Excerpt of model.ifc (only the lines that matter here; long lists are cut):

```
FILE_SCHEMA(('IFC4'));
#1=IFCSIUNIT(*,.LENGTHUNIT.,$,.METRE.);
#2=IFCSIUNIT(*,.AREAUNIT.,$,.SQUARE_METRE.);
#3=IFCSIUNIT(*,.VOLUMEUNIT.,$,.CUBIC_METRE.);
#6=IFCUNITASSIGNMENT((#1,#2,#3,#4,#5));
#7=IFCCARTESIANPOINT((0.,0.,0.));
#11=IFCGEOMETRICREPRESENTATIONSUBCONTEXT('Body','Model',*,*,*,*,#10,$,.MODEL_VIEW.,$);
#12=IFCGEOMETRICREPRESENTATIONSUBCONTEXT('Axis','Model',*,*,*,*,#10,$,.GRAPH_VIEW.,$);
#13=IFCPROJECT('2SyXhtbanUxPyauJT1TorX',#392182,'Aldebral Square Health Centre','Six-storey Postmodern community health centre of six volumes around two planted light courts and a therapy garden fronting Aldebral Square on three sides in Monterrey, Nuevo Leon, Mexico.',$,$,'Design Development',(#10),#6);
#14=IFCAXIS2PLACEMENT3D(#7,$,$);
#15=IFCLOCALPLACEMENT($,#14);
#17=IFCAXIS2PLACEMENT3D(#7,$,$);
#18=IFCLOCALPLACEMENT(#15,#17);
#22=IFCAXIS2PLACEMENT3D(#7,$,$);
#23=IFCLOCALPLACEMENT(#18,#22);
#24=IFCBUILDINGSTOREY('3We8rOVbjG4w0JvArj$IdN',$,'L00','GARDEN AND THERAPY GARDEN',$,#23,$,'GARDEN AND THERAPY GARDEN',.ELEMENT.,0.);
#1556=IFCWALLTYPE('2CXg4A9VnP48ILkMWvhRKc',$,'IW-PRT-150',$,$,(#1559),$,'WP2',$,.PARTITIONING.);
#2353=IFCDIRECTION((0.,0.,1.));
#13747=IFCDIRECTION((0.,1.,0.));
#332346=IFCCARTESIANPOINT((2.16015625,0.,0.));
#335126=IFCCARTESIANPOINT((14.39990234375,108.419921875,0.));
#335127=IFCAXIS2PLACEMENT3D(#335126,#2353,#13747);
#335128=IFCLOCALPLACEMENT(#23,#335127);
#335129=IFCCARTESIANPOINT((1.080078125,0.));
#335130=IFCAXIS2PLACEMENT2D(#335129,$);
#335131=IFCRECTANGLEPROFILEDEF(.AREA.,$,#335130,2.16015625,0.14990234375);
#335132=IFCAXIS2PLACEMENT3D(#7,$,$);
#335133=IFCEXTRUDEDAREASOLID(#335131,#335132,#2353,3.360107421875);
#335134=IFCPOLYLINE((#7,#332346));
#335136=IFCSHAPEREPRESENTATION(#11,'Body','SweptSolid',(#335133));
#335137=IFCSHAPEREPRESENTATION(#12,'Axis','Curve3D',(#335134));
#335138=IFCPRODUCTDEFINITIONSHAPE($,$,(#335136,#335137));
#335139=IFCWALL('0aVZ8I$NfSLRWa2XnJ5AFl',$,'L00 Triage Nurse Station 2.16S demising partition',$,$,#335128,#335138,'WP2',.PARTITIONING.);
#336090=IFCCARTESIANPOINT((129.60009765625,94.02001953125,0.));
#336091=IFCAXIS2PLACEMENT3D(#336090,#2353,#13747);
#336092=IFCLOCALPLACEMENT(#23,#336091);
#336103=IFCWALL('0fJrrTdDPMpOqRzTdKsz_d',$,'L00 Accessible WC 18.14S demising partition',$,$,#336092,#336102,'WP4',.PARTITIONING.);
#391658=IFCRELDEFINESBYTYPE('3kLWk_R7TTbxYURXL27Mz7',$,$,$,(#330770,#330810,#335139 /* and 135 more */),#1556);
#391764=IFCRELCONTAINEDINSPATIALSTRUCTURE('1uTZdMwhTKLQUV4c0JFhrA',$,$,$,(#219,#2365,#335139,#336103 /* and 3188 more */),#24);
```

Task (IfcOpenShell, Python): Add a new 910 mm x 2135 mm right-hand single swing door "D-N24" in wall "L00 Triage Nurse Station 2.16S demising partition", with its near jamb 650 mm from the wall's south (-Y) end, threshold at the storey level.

```python
import numpy as np
import ifcopenshell
import ifcopenshell.api.feature
import ifcopenshell.api.geometry
import ifcopenshell.api.root
import ifcopenshell.api.spatial
import ifcopenshell.geom
import ifcopenshell.util.element
import ifcopenshell.util.placement
import ifcopenshell.util.representation
import ifcopenshell.util.shape
import ifcopenshell.util.unit

model = ifcopenshell.open("model.ifc")
unit_scale = ifcopenshell.util.unit.calculate_unit_scale(model)
settings = ifcopenshell.geom.settings()


def volume(element):
    """Net volume in cubic metres, openings subtracted."""
    shape = ifcopenshell.geom.create_shape(settings, element)
    return ifcopenshell.util.shape.get_volume(shape.geometry)


wall = model.by_id(335139)
storey = ifcopenshell.util.element.get_container(wall, ifc_class="IfcBuildingStorey")
context = ifcopenshell.util.representation.get_context(model, "Model", "Body", "MODEL_VIEW")
before = volume(wall)

width, height, from_end, sill = 0.91, 2.135, 0.65, 0.0  # metres

# The wall runs along its own X axis, and the end named is its -X end.
wall_shape = ifcopenshell.geom.create_shape(settings, wall)
x, y, z = ifcopenshell.util.shape.get_vertices(wall_shape.geometry).T
start = x.min() + from_end
face, thickness = float(y.min()), float(y.max() - y.min())
wall_matrix = ifcopenshell.util.placement.get_local_placement(wall.ObjectPlacement)
level = ifcopenshell.util.placement.get_local_placement(storey.ObjectPlacement)[2, 3]


def in_wall(x, y):
    """Placement at x, y metres in the wall's axes, at sill height."""
    matrix = wall_matrix.copy()
    matrix[:, 3] = wall_matrix @ np.array([x / unit_scale, y / unit_scale, 0.0, 1.0])
    matrix[2, 3] = level + sill / unit_scale
    return matrix


# Opening: a box that overshoots both wall faces by 50 mm.
opening = ifcopenshell.api.root.create_entity(model, ifc_class="IfcOpeningElement", predefined_type="OPENING")
box = ifcopenshell.api.geometry.add_wall_representation(
    model, context=context, length=width, height=height, thickness=thickness + 0.1
)
ifcopenshell.api.geometry.assign_representation(model, product=opening, representation=box)
ifcopenshell.api.geometry.edit_object_placement(model, product=opening, matrix=in_wall(start, face - 0.05), is_si=False)
ifcopenshell.api.feature.add_feature(model, feature=opening, element=wall)

door = ifcopenshell.api.root.create_entity(model, ifc_class="IfcDoor", name="D-N24", predefined_type="DOOR")
door.OverallWidth, door.OverallHeight = width / unit_scale, height / unit_scale
door.OperationType = "SINGLE_SWING_RIGHT"
body = ifcopenshell.api.geometry.add_door_representation(
    model,
    context=context,
    overall_width=door.OverallWidth,
    overall_height=door.OverallHeight,
    operation_type="SINGLE_SWING_RIGHT",
    lining_properties={"LiningDepth": thickness / unit_scale, "ThresholdDepth": thickness / unit_scale},
)
ifcopenshell.api.geometry.assign_representation(model, product=door, representation=body)
ifcopenshell.api.spatial.assign_container(model, products=[door], relating_structure=storey)
ifcopenshell.api.feature.add_filling(model, opening=opening, element=door)

# The lining spans the wall, so the door starts at the wall face.
ifcopenshell.api.geometry.edit_object_placement(model, product=door, matrix=in_wall(start, face), is_si=False)

after = volume(wall)

print(f"wall volume {before:.3f} -> {after:.3f} m3")

model.write("model_edited.ifc")
```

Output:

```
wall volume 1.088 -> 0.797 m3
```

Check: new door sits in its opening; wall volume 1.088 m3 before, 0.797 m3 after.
